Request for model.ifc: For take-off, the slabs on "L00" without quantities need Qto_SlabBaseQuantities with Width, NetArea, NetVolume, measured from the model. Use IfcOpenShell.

First a look at what the model holds.

```python
import ifcopenshell
import ifcopenshell.util.element
import ifcopenshell.util.unit

model = ifcopenshell.open("model.ifc")
print(model.schema)
for unit_type in ("LENGTHUNIT", "AREAUNIT", "VOLUMEUNIT"):
    print(unit_type, ifcopenshell.util.unit.calculate_unit_scale(model, unit_type))
storey = next(s for s in model.by_type("IfcBuildingStorey") if s.Name == "L00")
slabs = [e for e in ifcopenshell.util.element.get_decomposition(storey) if e.is_a("IfcSlab")]
for e in sorted(slabs, key=lambda e: e.id()):
    print(e.id(), e.is_a(), e.Name, list(ifcopenshell.util.element.get_psets(e, qtos_only=True)), sep=" | ")
```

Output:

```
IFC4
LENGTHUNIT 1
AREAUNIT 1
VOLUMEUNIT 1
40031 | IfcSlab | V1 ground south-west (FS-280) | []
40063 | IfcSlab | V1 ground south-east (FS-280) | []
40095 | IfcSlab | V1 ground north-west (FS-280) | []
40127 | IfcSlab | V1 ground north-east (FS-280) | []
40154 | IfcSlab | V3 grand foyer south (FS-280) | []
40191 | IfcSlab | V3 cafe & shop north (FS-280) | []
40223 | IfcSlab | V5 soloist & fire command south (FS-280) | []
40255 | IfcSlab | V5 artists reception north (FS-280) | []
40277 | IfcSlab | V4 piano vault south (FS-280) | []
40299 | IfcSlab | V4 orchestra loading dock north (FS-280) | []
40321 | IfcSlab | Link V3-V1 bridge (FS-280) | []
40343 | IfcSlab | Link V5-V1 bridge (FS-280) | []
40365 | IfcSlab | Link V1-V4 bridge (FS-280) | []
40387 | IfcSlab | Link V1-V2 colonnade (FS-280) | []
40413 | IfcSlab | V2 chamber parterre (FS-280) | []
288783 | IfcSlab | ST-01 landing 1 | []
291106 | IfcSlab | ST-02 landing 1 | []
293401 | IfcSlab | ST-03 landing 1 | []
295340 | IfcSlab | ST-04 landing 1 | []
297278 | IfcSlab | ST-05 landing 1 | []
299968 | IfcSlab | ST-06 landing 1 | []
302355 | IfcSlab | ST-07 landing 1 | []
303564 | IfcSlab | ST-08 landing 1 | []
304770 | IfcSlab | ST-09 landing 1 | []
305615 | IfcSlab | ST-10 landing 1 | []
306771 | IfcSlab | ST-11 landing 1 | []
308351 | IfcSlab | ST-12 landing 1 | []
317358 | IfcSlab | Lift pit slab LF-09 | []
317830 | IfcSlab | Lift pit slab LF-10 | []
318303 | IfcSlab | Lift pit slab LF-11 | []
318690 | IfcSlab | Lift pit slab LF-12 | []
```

```python
import ifcopenshell
import ifcopenshell.api.pset
import ifcopenshell.geom
import ifcopenshell.util.element
import ifcopenshell.util.shape
import ifcopenshell.util.unit

model = ifcopenshell.open("model.ifc")
unit_scale = ifcopenshell.util.unit.calculate_unit_scale(model)
area_scale = ifcopenshell.util.unit.calculate_unit_scale(model, "AREAUNIT")
volume_scale = ifcopenshell.util.unit.calculate_unit_scale(model, "VOLUMEUNIT")
settings = ifcopenshell.geom.settings()

storey = next(s for s in model.by_type("IfcBuildingStorey") if s.Name == "L00")
slabs = [e for e in ifcopenshell.util.element.get_decomposition(storey) if e.is_a("IfcSlab")]

for e in sorted(slabs, key=lambda e: e.id()):
    if ifcopenshell.util.element.get_psets(e, qtos_only=True, should_inherit=False):
        continue
    # Geometry comes back in metres, in the element's own axes.
    shape = ifcopenshell.geom.create_shape(settings, e)
    values = {
        "Width": ifcopenshell.util.shape.get_z(shape.geometry) / unit_scale,
        "NetArea": ifcopenshell.util.shape.get_footprint_area(shape.geometry) / area_scale,
        "NetVolume": ifcopenshell.util.shape.get_volume(shape.geometry) / volume_scale,
    }
    qto = ifcopenshell.api.pset.add_qto(model, product=e, name="Qto_SlabBaseQuantities")
    ifcopenshell.api.pset.edit_qto(model, qto=qto, properties=values)
    print(e.id(), {k: round(v, 3) for k, v in values.items()})

model.write("model_updated.ifc")
```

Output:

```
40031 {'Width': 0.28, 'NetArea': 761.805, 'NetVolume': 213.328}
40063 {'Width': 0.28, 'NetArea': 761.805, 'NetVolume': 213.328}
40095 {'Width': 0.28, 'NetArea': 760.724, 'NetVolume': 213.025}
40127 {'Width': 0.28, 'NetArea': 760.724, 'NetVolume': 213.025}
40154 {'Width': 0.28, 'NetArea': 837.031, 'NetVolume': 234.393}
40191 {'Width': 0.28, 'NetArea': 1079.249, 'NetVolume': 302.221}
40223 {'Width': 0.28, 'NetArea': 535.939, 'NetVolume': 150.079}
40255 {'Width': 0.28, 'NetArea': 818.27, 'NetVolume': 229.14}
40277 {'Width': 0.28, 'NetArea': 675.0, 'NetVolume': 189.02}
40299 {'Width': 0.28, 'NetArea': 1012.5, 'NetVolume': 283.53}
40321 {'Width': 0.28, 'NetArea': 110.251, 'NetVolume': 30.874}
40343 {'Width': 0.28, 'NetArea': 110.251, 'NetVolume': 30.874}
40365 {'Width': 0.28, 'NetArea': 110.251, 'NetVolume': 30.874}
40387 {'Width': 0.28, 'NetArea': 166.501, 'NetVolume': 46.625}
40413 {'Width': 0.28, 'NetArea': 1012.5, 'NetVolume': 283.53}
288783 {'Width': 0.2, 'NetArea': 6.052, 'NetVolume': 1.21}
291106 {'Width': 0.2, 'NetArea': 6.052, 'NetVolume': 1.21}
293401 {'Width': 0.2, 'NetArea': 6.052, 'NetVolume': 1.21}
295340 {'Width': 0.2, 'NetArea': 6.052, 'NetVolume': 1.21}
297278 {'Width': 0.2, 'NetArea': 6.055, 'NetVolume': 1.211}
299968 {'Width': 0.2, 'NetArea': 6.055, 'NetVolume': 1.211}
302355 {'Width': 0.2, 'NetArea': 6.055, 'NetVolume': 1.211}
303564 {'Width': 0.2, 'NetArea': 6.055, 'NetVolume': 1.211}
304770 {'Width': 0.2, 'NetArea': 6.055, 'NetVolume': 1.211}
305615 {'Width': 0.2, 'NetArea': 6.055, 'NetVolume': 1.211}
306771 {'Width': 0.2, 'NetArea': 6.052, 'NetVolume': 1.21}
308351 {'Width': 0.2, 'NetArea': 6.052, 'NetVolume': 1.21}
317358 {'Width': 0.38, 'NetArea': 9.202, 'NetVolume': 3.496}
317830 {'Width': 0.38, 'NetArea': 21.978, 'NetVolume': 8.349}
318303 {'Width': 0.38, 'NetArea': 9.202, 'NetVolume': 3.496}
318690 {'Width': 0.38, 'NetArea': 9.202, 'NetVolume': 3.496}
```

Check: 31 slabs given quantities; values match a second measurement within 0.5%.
